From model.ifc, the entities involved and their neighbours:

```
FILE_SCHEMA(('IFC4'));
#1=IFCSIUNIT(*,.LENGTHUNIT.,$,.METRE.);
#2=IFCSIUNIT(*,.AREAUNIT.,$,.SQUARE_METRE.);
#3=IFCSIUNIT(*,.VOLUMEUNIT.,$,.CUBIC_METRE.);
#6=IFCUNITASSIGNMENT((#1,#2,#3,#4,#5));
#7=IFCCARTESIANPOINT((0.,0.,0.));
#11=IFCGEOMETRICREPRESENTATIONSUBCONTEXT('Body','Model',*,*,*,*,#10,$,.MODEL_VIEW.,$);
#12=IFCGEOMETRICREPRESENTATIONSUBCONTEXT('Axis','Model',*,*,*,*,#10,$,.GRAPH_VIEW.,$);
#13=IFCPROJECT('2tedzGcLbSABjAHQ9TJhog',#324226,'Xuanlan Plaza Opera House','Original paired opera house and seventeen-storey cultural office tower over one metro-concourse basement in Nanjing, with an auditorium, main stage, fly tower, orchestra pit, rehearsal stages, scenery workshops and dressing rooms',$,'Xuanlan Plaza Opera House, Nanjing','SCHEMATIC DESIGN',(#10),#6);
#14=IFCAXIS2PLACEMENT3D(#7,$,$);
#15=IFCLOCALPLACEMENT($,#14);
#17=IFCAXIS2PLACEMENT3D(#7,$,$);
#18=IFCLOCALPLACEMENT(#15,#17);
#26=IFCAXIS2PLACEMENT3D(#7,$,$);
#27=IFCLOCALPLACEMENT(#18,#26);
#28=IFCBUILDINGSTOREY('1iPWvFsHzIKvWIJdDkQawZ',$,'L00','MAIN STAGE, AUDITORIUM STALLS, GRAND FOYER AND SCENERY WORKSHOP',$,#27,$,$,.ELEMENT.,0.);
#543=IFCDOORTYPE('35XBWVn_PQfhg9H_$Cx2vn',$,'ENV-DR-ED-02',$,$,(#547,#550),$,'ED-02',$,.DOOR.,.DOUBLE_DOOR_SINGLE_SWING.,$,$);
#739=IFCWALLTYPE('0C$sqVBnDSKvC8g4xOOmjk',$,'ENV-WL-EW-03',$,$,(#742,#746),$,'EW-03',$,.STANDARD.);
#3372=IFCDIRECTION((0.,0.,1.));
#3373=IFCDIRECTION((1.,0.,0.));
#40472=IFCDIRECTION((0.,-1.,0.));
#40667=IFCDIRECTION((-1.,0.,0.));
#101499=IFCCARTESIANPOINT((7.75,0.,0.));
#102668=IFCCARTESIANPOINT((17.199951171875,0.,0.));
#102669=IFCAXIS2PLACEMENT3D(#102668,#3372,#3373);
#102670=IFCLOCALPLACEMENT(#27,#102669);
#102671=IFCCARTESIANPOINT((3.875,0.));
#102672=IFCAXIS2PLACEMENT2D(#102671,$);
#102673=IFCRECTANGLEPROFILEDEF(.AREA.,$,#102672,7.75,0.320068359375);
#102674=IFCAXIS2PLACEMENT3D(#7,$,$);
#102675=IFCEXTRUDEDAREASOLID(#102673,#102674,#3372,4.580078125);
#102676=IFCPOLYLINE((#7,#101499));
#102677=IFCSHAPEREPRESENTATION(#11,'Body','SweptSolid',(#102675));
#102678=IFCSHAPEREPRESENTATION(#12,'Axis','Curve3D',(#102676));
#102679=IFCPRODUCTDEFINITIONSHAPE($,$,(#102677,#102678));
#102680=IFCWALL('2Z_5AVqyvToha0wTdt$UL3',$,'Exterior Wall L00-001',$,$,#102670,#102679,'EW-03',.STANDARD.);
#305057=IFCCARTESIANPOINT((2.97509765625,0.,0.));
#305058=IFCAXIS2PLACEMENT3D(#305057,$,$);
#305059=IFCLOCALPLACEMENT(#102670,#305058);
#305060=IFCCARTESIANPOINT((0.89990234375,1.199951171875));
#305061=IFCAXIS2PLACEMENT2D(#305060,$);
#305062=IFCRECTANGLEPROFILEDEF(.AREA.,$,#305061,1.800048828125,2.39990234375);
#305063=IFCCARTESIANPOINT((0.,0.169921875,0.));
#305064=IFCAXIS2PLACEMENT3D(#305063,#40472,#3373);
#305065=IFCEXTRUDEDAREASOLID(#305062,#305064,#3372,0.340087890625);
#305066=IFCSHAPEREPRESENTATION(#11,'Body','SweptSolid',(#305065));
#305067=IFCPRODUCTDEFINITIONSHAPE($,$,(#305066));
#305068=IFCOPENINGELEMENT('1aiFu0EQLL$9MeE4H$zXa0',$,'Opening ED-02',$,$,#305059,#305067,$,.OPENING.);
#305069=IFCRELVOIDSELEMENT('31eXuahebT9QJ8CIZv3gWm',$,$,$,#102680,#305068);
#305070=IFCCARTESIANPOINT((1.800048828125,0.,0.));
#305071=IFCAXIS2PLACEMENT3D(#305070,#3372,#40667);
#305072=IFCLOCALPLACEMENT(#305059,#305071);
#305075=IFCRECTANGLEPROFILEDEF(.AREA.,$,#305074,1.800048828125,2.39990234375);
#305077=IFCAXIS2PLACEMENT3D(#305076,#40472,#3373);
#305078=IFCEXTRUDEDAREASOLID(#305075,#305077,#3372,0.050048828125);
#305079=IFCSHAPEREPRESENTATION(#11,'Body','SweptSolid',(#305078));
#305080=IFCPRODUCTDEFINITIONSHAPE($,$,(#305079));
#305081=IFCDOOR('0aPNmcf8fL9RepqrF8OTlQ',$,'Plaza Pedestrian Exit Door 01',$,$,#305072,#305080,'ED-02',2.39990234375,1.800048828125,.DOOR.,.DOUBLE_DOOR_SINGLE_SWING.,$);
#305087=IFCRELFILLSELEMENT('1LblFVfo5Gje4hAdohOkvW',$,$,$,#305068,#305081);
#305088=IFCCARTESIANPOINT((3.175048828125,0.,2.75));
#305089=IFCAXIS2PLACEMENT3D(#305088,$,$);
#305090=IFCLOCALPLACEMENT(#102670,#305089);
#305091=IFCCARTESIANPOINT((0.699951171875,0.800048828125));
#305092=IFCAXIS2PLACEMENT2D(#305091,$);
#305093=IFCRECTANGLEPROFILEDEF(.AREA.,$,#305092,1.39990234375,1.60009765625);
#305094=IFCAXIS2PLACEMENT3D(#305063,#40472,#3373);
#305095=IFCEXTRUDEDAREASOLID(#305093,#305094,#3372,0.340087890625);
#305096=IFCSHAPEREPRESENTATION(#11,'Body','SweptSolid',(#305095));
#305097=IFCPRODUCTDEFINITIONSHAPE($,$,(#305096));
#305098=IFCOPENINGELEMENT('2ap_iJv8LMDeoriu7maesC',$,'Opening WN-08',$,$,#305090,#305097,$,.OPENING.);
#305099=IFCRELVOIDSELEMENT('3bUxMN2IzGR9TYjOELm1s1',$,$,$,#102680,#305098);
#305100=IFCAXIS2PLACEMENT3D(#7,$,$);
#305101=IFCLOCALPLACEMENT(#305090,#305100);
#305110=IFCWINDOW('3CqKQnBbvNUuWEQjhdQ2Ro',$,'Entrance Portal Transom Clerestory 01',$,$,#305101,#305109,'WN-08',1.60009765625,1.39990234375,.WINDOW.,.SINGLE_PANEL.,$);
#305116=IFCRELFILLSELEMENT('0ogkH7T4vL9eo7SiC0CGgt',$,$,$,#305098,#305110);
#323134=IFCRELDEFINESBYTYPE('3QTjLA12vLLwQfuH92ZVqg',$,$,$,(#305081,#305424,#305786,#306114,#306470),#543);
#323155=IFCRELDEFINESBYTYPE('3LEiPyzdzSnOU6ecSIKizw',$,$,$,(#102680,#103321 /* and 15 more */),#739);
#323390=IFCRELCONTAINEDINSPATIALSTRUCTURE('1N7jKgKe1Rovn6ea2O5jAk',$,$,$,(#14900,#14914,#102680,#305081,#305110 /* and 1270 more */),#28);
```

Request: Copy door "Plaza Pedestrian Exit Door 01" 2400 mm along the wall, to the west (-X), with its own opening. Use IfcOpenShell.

```python
import ifcopenshell
import ifcopenshell.api.feature
import ifcopenshell.api.geometry
import ifcopenshell.api.root
import ifcopenshell.geom
import ifcopenshell.util.element
import ifcopenshell.util.placement
import ifcopenshell.util.shape
import ifcopenshell.util.unit

model = ifcopenshell.open("model.ifc")
unit_scale = ifcopenshell.util.unit.calculate_unit_scale(model)
settings = ifcopenshell.geom.settings()


def volume(element):
    """Net volume in cubic metres, openings subtracted."""
    shape = ifcopenshell.geom.create_shape(settings, element)
    return ifcopenshell.util.shape.get_volume(shape.geometry)


door = model.by_id(305081)
opening = door.FillsVoids[0].RelatingOpeningElement
wall = opening.VoidsElements[0].RelatingBuildingElement
before = volume(wall)
shift = ifcopenshell.util.placement.get_local_placement(wall.ObjectPlacement)[:3, 0] * -2.4 / unit_scale

# copy_class copies the void relationship, type, container and properties, but no geometry.
new_opening = ifcopenshell.api.root.copy_class(model, product=opening)
new_opening.Representation = ifcopenshell.util.element.copy_deep(
    model, opening.Representation, exclude=["IfcGeometricRepresentationContext", "IfcRepresentationMap"]
)
new_door = ifcopenshell.api.root.copy_class(model, product=door)
new_door.Representation = ifcopenshell.util.element.copy_deep(
    model, door.Representation, exclude=["IfcGeometricRepresentationContext", "IfcRepresentationMap"]
)
new_door.Tag = None
ifcopenshell.api.feature.add_filling(model, opening=new_opening, element=new_door)

for old, new in ((opening, new_opening), (door, new_door)):
    matrix = ifcopenshell.util.placement.get_local_placement(old.ObjectPlacement)
    matrix[:3, 3] += shift
    ifcopenshell.api.geometry.edit_object_placement(model, product=new, matrix=matrix, is_si=False)

after = volume(wall)

print(f"wall volume {before:.3f} -> {after:.3f} m3")

model.write("model_updated.ifc")
```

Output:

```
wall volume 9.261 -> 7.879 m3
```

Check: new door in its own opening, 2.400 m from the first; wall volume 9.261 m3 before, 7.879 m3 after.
